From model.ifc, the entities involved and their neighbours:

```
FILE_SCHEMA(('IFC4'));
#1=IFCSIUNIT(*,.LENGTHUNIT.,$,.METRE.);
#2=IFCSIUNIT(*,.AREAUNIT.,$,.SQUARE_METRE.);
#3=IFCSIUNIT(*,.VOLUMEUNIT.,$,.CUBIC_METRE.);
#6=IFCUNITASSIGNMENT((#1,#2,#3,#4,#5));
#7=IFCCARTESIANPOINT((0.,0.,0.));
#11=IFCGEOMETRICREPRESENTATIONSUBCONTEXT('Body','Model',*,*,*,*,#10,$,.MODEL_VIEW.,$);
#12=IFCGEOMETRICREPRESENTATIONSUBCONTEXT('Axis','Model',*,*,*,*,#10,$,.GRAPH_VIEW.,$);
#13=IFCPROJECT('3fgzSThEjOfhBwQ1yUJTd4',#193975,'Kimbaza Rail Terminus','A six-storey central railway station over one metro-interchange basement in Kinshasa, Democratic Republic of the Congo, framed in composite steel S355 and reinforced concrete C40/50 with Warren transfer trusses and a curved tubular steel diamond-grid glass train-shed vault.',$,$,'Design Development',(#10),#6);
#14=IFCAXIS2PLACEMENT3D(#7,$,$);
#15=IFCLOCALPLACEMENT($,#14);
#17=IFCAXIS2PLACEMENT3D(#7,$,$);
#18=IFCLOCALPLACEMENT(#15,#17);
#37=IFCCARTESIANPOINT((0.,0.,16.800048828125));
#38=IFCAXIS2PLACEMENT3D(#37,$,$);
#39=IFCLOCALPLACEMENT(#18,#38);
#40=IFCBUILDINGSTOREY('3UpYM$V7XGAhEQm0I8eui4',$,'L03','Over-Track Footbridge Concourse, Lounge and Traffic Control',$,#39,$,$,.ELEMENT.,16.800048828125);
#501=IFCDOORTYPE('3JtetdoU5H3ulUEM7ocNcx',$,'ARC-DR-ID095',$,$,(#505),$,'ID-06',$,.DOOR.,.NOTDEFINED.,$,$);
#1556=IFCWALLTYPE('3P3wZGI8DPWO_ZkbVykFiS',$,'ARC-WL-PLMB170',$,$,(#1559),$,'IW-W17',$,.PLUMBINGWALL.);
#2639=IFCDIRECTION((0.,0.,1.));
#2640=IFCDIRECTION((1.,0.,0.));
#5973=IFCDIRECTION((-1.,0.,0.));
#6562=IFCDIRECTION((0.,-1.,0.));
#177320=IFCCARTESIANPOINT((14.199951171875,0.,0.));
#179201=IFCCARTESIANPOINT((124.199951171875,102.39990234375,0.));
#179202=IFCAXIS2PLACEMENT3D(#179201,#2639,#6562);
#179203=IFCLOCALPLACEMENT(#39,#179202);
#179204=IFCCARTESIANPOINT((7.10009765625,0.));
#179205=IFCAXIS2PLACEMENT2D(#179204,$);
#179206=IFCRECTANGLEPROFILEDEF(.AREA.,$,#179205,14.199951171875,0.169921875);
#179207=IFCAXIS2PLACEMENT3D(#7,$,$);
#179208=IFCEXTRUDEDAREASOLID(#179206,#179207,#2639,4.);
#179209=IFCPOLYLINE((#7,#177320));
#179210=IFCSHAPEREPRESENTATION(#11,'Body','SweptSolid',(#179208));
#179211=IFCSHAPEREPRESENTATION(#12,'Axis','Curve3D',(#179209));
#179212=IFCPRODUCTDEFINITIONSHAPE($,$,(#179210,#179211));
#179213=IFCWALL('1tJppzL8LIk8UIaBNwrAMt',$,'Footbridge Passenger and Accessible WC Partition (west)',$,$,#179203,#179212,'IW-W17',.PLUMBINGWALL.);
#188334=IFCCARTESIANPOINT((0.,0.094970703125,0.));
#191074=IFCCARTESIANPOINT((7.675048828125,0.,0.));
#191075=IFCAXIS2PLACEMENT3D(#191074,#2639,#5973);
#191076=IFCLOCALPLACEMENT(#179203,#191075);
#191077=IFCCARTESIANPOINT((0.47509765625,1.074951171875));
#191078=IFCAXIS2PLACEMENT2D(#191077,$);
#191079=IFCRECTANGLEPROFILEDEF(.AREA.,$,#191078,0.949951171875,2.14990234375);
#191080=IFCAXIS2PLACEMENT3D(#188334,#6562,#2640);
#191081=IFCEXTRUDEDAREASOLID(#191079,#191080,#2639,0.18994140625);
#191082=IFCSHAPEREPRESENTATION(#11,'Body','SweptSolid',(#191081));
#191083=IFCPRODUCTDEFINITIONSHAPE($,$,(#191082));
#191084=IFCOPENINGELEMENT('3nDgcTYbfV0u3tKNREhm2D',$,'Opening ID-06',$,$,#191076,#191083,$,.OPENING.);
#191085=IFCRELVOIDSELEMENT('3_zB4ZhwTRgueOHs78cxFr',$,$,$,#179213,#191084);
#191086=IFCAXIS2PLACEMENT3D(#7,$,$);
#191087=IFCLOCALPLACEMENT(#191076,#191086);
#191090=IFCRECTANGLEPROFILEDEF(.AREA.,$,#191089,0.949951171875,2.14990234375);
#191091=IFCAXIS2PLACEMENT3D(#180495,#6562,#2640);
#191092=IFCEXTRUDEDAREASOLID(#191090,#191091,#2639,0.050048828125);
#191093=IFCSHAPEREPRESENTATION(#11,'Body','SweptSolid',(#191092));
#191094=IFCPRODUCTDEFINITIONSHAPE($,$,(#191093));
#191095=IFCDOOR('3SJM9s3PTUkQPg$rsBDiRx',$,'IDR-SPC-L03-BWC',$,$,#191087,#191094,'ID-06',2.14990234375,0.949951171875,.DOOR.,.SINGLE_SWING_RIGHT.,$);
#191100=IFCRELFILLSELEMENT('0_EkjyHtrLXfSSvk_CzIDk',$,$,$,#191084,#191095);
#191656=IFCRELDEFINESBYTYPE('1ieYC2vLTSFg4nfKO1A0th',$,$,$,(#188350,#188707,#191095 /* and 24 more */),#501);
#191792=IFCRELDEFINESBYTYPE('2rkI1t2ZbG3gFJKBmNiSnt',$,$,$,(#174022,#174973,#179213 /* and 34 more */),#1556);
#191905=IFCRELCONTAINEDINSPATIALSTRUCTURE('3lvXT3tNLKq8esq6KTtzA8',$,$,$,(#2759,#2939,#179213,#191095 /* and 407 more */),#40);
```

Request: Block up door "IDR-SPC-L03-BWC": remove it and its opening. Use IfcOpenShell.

```python
import ifcopenshell
import ifcopenshell.api.feature
import ifcopenshell.api.root
import ifcopenshell.geom
import ifcopenshell.util.shape

model = ifcopenshell.open("model.ifc")
settings = ifcopenshell.geom.settings()


def volume(element):
    """Net volume in cubic metres, openings subtracted."""
    shape = ifcopenshell.geom.create_shape(settings, element)
    return ifcopenshell.util.shape.get_volume(shape.geometry)


door = model.by_guid("3SJM9s3PTUkQPg$rsBDiRx")
opening = door.FillsVoids[0].RelatingOpeningElement
wall = opening.VoidsElements[0].RelatingBuildingElement
before = volume(wall)

ifcopenshell.api.root.remove_product(model, product=door)
ifcopenshell.api.feature.remove_feature(model, feature=opening)

after = volume(wall)

print(f"wall volume {before:.3f} -> {after:.3f} m3")

model.write("model_rev.ifc")
```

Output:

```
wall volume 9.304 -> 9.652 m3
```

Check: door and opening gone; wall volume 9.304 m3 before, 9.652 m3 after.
